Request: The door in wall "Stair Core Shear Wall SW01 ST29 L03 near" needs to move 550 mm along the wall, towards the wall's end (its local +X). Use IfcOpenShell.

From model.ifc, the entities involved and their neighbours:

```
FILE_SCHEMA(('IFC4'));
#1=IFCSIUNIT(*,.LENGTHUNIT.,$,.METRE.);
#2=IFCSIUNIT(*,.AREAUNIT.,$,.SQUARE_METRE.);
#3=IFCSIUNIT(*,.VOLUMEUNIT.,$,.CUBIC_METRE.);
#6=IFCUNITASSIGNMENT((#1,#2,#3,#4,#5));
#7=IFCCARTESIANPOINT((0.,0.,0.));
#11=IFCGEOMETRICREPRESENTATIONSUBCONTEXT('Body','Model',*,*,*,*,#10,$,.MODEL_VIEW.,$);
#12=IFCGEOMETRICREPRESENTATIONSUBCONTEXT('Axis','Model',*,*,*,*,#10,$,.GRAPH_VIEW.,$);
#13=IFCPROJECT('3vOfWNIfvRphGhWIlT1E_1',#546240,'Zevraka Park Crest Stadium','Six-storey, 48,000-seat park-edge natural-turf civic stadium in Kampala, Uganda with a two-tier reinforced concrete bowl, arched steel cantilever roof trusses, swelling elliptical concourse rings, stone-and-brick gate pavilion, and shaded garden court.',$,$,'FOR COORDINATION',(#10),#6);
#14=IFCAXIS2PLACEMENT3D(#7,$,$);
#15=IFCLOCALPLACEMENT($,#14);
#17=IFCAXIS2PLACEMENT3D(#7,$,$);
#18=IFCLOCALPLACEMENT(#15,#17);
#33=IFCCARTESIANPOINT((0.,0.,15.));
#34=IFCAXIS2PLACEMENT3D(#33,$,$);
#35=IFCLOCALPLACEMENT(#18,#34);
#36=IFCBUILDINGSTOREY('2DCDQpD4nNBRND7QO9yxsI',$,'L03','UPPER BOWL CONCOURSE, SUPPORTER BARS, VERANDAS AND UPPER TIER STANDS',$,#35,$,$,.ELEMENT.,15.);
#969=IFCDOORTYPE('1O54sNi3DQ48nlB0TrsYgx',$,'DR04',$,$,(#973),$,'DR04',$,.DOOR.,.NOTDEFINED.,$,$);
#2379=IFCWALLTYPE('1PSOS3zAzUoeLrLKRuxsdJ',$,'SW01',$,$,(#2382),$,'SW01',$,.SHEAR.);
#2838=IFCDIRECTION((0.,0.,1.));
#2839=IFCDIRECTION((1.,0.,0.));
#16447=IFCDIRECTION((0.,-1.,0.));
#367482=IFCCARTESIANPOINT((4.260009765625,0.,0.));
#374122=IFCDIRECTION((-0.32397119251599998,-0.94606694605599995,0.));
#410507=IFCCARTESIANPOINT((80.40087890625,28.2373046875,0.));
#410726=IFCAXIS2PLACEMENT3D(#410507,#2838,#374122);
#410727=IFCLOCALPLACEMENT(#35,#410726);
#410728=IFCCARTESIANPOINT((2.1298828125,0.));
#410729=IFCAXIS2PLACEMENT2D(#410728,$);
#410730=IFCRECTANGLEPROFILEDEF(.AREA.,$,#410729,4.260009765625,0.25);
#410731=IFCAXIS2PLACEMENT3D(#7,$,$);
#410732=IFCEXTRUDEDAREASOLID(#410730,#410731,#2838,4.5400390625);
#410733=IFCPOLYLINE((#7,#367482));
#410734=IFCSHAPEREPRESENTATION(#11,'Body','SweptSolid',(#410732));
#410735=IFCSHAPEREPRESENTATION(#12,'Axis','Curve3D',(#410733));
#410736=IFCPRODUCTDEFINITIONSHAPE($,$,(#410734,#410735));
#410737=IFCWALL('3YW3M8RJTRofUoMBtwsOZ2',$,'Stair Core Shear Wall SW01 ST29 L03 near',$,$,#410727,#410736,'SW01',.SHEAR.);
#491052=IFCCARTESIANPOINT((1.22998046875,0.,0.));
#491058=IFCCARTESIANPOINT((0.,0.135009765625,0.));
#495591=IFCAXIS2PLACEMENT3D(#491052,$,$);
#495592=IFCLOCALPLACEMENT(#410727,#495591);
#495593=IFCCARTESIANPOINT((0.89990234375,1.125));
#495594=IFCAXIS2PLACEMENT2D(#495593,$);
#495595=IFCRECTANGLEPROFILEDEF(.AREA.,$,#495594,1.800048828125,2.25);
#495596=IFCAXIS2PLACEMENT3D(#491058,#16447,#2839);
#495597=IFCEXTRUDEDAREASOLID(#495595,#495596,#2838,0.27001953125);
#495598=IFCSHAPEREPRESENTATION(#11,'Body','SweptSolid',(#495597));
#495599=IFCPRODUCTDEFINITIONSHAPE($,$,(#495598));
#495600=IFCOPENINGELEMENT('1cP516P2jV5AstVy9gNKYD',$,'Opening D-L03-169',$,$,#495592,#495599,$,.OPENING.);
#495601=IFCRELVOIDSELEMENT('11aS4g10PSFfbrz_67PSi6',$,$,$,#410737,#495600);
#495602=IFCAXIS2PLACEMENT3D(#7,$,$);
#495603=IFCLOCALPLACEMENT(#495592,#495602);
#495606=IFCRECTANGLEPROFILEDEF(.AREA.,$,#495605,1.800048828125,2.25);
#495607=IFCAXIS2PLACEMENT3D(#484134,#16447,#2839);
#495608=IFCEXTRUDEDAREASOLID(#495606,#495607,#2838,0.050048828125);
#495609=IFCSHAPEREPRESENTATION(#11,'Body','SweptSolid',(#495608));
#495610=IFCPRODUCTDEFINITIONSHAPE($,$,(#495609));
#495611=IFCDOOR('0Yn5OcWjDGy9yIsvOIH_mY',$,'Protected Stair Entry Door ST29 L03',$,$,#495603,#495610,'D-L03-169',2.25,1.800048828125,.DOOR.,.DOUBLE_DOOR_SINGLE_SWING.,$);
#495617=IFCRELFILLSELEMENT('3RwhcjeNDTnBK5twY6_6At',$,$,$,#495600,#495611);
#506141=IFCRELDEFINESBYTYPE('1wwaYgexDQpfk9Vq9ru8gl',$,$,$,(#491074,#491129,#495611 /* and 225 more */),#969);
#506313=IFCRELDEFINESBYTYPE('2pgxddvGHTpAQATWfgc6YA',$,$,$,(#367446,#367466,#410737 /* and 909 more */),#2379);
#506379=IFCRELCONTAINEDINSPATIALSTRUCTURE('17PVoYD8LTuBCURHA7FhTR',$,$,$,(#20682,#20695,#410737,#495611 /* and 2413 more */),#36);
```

```python
import ifcopenshell
import ifcopenshell.api.geometry
import ifcopenshell.util.placement
import ifcopenshell.util.unit

model = ifcopenshell.open("model.ifc")
unit_scale = ifcopenshell.util.unit.calculate_unit_scale(model)

door = model.by_guid("0Yn5OcWjDGy9yIsvOIH_mY")
opening = door.FillsVoids[0].RelatingOpeningElement
wall = opening.VoidsElements[0].RelatingBuildingElement

wall_matrix = ifcopenshell.util.placement.get_local_placement(wall.ObjectPlacement)
shift = wall_matrix[:3, 0] * 0.55 / unit_scale
before = ifcopenshell.util.placement.get_local_placement(door.ObjectPlacement)[:3, 3].copy()

# The door is placed relative to its opening, so it follows when the opening moves.
matrix = ifcopenshell.util.placement.get_local_placement(opening.ObjectPlacement)
matrix[:3, 3] += shift
ifcopenshell.api.geometry.edit_object_placement(
    model, product=opening, matrix=matrix, is_si=False, should_transform_children=True
)

after = ifcopenshell.util.placement.get_local_placement(door.ObjectPlacement)[:3, 3]
print("door moved by", (after - before).round(3) + 0.0)

model.write("model-out.ifc")
```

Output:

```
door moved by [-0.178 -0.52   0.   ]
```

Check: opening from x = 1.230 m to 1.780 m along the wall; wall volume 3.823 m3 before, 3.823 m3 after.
